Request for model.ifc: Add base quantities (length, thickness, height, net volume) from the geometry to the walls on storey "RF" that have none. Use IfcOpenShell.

First a look at what the model holds.

```python
import ifcopenshell
import ifcopenshell.util.element
import ifcopenshell.util.unit

model = ifcopenshell.open("model.ifc")
print(model.schema)
for unit_type in ("LENGTHUNIT", "AREAUNIT", "VOLUMEUNIT"):
    print(unit_type, ifcopenshell.util.unit.calculate_unit_scale(model, unit_type))
storey = next(s for s in model.by_type("IfcBuildingStorey") if s.Name == "RF")
walls = [e for e in ifcopenshell.util.element.get_decomposition(storey) if e.is_a("IfcWall")]
for e in sorted(walls, key=lambda e: e.id()):
    print(e.id(), e.is_a(), e.Name, list(ifcopenshell.util.element.get_psets(e, qtos_only=True)), sep=" | ")
```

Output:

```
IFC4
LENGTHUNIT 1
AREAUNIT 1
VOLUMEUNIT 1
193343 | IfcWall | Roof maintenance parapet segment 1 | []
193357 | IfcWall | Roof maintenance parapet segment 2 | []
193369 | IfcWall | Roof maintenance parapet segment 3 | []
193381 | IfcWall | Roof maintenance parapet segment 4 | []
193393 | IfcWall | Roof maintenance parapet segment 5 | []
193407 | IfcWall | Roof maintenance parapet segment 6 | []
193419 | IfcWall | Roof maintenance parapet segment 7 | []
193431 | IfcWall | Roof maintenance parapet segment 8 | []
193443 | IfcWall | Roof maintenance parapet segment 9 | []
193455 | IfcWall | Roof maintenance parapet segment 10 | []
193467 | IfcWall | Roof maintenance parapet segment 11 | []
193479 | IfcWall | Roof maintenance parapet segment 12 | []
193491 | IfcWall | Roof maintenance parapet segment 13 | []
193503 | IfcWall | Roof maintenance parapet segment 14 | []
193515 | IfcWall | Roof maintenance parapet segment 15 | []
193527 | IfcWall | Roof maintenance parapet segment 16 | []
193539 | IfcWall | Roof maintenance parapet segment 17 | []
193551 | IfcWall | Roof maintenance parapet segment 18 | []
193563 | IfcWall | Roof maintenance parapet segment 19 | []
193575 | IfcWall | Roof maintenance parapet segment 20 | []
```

```python
import ifcopenshell
import ifcopenshell.api.pset
import ifcopenshell.geom
import ifcopenshell.util.element
import ifcopenshell.util.shape
import ifcopenshell.util.unit

model = ifcopenshell.open("model.ifc")
unit_scale = ifcopenshell.util.unit.calculate_unit_scale(model)
volume_scale = ifcopenshell.util.unit.calculate_unit_scale(model, "VOLUMEUNIT")
settings = ifcopenshell.geom.settings()

storey = next(s for s in model.by_type("IfcBuildingStorey") if s.Name == "RF")
walls = [e for e in ifcopenshell.util.element.get_decomposition(storey) if e.is_a("IfcWall")]

for e in sorted(walls, key=lambda e: e.id()):
    if ifcopenshell.util.element.get_psets(e, qtos_only=True, should_inherit=False):
        continue
    # Geometry comes back in metres, in the element's own axes.
    shape = ifcopenshell.geom.create_shape(settings, e)
    values = {
        "Length": ifcopenshell.util.shape.get_x(shape.geometry) / unit_scale,
        "Width": ifcopenshell.util.shape.get_y(shape.geometry) / unit_scale,
        "Height": ifcopenshell.util.shape.get_z(shape.geometry) / unit_scale,
        "NetVolume": ifcopenshell.util.shape.get_volume(shape.geometry) / volume_scale,
    }
    qto = ifcopenshell.api.pset.add_qto(model, product=e, name="Qto_WallBaseQuantities")
    ifcopenshell.api.pset.edit_qto(model, qto=qto, properties=values)
    print(e.id(), {k: round(v, 3) for k, v in values.items()})

model.write("model_rev.ifc")
```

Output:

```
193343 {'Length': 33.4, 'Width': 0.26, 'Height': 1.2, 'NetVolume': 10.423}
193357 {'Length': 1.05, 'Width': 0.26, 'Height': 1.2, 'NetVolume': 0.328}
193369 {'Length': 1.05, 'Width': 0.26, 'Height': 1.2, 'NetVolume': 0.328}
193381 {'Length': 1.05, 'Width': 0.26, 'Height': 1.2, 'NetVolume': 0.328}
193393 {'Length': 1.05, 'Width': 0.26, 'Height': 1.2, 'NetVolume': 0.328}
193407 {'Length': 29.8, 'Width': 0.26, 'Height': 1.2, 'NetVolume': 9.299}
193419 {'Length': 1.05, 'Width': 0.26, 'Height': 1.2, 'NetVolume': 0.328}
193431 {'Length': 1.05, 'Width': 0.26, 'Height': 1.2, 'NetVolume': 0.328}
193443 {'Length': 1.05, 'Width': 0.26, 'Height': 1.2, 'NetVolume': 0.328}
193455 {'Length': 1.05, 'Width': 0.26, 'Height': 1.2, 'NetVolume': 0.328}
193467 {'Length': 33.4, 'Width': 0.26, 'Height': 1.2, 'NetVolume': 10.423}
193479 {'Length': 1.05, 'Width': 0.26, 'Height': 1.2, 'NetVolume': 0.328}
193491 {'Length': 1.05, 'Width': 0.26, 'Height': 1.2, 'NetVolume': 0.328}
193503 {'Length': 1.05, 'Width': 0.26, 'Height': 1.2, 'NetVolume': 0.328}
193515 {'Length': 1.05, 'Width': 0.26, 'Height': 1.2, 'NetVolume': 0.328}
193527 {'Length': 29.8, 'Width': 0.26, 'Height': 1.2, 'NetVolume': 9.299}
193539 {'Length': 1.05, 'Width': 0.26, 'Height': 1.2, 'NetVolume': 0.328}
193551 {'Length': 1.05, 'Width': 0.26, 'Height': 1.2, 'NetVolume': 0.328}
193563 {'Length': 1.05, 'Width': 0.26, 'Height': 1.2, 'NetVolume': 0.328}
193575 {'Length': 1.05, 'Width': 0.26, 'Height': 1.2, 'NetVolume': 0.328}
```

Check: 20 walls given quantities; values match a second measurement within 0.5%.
